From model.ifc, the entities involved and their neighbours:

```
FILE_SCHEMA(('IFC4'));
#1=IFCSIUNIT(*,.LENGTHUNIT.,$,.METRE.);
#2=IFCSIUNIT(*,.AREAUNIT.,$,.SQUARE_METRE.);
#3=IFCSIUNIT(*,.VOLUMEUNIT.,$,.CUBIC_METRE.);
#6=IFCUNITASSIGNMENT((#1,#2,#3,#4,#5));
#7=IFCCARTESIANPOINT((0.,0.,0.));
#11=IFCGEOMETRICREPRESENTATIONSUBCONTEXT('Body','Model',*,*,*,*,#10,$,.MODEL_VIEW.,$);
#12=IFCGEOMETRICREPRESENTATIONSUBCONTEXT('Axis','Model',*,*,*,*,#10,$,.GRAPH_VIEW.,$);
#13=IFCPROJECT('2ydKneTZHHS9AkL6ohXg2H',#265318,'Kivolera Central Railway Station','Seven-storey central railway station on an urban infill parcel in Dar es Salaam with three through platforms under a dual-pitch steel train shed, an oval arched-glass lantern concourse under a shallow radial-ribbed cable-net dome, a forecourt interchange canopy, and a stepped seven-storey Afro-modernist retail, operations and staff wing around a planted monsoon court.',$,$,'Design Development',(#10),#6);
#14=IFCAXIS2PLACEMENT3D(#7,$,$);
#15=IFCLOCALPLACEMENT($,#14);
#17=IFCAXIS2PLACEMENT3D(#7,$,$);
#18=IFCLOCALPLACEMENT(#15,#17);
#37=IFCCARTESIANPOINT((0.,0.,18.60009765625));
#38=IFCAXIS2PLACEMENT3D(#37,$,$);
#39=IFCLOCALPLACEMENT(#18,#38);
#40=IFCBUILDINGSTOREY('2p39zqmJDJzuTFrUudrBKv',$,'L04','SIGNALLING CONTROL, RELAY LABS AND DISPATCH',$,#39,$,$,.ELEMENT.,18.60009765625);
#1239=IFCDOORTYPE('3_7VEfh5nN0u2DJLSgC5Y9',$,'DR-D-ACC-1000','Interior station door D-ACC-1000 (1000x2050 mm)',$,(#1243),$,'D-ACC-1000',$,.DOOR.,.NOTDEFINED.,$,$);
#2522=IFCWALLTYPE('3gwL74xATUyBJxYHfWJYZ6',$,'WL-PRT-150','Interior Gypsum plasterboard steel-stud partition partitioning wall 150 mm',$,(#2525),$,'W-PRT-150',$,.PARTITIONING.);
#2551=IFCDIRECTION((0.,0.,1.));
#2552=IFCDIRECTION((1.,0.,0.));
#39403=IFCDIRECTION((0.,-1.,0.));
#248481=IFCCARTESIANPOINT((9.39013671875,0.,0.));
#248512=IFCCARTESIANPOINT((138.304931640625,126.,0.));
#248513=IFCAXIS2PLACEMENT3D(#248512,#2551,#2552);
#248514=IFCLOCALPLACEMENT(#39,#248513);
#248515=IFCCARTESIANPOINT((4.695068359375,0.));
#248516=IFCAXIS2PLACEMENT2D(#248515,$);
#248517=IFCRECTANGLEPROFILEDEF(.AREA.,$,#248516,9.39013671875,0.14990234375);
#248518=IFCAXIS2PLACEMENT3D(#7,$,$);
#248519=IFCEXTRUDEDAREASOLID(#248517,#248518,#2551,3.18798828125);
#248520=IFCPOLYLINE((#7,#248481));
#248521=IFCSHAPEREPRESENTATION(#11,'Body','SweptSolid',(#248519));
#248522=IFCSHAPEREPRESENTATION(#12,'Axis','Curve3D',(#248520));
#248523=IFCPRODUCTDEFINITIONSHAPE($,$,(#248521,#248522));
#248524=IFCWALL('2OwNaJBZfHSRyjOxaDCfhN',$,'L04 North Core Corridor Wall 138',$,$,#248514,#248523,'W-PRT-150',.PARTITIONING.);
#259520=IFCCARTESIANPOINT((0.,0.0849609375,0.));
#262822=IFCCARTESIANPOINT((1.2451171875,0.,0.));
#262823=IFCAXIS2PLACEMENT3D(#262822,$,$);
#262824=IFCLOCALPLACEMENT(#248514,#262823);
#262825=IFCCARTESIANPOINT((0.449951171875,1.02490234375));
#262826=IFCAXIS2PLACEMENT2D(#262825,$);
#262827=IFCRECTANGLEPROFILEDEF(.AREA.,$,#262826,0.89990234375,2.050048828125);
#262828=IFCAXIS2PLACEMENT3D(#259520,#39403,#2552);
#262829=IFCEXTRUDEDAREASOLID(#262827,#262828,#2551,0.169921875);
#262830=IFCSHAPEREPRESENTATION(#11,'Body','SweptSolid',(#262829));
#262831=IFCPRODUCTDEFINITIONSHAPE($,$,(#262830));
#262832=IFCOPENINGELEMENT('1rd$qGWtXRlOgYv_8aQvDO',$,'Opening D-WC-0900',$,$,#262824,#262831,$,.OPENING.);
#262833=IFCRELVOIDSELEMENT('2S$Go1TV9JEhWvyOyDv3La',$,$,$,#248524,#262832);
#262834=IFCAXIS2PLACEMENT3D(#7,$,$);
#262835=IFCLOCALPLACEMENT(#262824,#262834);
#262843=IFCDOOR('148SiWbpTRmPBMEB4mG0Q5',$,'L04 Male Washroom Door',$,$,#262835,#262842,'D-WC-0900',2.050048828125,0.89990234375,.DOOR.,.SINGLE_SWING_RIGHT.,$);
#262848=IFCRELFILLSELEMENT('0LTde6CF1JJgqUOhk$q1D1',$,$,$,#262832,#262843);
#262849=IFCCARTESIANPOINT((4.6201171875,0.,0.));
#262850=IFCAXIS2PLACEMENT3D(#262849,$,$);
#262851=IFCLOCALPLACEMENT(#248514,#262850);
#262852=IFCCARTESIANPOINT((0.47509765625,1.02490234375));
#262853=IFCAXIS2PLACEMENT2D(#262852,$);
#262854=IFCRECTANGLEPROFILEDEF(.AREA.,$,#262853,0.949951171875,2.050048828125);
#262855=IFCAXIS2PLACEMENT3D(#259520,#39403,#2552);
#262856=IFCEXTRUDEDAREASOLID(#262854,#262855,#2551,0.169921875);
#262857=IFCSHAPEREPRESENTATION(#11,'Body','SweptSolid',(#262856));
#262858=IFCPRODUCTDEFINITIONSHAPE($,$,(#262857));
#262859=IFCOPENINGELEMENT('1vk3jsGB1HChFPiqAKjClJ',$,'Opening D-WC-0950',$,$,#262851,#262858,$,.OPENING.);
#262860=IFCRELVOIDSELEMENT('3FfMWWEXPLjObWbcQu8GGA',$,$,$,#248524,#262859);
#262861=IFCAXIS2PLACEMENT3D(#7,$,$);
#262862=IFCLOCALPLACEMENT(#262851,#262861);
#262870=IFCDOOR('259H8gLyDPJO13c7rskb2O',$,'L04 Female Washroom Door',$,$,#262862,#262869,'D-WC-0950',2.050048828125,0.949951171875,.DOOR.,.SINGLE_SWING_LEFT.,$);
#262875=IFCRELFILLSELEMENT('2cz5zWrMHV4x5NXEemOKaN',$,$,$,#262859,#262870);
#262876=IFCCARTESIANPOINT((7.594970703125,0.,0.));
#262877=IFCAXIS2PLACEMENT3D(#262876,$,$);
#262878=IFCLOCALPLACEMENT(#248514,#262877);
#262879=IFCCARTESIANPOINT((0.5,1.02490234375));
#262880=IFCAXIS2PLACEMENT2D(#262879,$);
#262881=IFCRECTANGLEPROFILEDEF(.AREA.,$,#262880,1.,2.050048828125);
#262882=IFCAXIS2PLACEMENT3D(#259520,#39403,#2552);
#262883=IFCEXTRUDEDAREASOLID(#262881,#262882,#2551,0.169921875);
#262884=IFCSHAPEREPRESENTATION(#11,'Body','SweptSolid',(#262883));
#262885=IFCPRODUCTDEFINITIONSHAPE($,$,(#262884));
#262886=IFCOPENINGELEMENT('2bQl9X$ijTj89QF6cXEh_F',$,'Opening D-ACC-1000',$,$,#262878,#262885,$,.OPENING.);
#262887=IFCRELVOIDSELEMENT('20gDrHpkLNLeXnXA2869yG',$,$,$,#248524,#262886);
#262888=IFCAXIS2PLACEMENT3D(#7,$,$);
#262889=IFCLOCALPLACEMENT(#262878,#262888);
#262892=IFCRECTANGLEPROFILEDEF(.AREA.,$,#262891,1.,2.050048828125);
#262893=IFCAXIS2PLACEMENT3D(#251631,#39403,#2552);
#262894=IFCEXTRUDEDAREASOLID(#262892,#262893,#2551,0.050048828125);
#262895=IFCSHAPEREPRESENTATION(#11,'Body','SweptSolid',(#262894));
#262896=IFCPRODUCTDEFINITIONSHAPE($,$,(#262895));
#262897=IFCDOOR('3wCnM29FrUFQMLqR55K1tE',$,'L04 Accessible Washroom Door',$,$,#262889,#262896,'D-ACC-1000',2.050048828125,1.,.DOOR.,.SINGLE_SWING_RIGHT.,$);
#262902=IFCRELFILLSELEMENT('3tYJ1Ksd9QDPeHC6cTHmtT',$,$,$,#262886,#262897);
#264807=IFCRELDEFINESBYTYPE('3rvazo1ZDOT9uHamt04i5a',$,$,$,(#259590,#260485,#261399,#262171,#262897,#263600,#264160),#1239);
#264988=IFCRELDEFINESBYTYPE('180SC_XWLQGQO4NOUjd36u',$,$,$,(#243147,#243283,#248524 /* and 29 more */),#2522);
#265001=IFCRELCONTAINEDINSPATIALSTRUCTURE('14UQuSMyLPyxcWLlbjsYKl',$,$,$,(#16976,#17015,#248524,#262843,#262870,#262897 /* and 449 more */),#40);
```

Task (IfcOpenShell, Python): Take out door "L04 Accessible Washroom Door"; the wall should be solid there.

```python
import ifcopenshell
import ifcopenshell.api.feature
import ifcopenshell.api.root
import ifcopenshell.geom
import ifcopenshell.util.shape

model = ifcopenshell.open("model.ifc")
settings = ifcopenshell.geom.settings()


def volume(element):
    """Net volume in cubic metres, openings subtracted."""
    shape = ifcopenshell.geom.create_shape(settings, element)
    return ifcopenshell.util.shape.get_volume(shape.geometry)


door = model.by_guid("3wCnM29FrUFQMLqR55K1tE")
opening = door.FillsVoids[0].RelatingOpeningElement
wall = opening.VoidsElements[0].RelatingBuildingElement
before = volume(wall)

ifcopenshell.api.root.remove_product(model, product=door)
ifcopenshell.api.feature.remove_feature(model, feature=opening)

after = volume(wall)

print(f"wall volume {before:.3f} -> {after:.3f} m3")

model.write("model-out.ifc")
```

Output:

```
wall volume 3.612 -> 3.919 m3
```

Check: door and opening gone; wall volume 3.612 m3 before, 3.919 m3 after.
